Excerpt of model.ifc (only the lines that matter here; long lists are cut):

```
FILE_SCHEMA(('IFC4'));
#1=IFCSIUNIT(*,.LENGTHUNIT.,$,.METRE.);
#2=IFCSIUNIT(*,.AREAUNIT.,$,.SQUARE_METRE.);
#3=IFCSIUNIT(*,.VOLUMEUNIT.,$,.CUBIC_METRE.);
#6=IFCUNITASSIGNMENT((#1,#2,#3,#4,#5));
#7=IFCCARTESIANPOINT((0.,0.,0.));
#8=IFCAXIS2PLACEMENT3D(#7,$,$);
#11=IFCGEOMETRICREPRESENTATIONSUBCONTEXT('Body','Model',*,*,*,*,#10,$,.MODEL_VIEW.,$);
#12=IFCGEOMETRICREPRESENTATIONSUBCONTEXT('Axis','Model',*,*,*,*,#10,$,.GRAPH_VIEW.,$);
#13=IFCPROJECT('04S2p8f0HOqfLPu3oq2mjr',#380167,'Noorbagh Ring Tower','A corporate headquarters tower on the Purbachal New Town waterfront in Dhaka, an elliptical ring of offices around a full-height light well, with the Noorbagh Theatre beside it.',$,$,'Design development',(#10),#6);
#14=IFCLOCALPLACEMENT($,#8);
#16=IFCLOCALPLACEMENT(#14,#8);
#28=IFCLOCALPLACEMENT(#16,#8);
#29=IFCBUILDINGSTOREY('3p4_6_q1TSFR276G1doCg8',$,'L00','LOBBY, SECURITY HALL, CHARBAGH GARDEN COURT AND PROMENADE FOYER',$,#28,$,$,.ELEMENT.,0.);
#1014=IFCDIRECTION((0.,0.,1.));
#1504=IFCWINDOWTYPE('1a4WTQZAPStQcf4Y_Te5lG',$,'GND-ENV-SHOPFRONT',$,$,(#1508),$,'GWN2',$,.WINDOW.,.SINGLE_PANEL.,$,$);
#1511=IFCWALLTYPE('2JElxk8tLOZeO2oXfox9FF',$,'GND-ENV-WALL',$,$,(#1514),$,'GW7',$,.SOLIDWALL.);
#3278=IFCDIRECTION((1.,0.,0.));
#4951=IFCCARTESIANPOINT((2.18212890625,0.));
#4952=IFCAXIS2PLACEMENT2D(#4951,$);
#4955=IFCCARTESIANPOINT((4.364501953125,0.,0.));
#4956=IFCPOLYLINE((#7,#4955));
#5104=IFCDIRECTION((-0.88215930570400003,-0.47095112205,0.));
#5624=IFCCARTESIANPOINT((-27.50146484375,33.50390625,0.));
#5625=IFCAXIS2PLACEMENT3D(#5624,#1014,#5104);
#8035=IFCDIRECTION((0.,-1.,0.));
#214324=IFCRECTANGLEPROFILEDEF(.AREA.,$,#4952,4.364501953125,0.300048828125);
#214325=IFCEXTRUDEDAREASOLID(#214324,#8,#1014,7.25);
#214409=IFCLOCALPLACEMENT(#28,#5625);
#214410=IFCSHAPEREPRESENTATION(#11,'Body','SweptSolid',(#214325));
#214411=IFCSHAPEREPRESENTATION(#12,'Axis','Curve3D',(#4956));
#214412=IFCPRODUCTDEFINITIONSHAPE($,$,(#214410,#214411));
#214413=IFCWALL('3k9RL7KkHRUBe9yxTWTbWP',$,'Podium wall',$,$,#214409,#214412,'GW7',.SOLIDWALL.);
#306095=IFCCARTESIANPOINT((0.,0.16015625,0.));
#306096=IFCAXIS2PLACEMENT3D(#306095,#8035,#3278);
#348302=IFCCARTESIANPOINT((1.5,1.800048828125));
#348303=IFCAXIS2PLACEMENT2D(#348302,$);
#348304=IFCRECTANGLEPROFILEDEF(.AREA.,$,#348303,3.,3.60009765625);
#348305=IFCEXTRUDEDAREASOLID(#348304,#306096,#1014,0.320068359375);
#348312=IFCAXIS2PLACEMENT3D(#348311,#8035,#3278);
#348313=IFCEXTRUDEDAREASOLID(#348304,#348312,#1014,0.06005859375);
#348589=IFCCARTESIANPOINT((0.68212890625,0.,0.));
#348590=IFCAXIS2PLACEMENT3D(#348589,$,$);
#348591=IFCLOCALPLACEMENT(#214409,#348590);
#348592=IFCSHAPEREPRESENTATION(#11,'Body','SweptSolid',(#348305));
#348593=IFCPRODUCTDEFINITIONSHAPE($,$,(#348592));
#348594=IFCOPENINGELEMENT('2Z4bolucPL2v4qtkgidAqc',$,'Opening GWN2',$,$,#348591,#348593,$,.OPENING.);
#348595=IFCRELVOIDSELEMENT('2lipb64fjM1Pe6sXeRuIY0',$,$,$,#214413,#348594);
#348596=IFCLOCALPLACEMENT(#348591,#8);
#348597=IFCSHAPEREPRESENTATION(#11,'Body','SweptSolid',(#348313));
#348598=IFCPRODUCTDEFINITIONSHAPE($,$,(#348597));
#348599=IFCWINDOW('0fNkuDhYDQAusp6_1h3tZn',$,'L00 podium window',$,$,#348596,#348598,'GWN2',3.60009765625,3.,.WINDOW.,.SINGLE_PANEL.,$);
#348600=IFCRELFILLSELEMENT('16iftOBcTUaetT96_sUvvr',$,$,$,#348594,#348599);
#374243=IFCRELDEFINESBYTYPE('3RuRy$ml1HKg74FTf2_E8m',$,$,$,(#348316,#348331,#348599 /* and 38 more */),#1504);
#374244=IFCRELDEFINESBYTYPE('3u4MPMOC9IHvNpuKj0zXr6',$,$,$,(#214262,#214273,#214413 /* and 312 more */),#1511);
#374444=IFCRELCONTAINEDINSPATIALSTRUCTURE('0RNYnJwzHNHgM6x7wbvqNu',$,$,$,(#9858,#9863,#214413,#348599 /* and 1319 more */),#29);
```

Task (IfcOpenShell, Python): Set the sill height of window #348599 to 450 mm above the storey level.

```python
import numpy as np
import ifcopenshell
import ifcopenshell.api.geometry
import ifcopenshell.geom
import ifcopenshell.util.element
import ifcopenshell.util.placement
import ifcopenshell.util.shape
import ifcopenshell.util.unit

model = ifcopenshell.open("model.ifc")
unit_scale = ifcopenshell.util.unit.calculate_unit_scale(model)

window = model.by_guid("0fNkuDhYDQAusp6_1h3tZn")
opening = window.FillsVoids[0].RelatingOpeningElement
storey = ifcopenshell.util.element.get_container(window, ifc_class="IfcBuildingStorey")
level = ifcopenshell.util.placement.get_local_placement(storey.ObjectPlacement)[2, 3]

# The opening's origin need not be at the sill, so measure its lowest point.
shape = ifcopenshell.geom.create_shape(ifcopenshell.geom.settings(), opening)
bottom = ifcopenshell.util.shape.get_shape_bottom_elevation(shape, shape.geometry) / unit_scale
dz = level + 0.45 - bottom

shift = np.array([0.0, 0.0, dz])
# The window is placed relative to its opening, so it follows when the opening moves.
matrix = ifcopenshell.util.placement.get_local_placement(opening.ObjectPlacement)
matrix[:3, 3] += shift
ifcopenshell.api.geometry.edit_object_placement(
    model, product=opening, matrix=matrix, is_si=False, should_transform_children=True
)

print(f"moved by {dz * unit_scale:+.3f} m")

model.write("model-out.ifc")
```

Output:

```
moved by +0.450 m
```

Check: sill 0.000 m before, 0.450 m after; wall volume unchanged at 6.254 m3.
